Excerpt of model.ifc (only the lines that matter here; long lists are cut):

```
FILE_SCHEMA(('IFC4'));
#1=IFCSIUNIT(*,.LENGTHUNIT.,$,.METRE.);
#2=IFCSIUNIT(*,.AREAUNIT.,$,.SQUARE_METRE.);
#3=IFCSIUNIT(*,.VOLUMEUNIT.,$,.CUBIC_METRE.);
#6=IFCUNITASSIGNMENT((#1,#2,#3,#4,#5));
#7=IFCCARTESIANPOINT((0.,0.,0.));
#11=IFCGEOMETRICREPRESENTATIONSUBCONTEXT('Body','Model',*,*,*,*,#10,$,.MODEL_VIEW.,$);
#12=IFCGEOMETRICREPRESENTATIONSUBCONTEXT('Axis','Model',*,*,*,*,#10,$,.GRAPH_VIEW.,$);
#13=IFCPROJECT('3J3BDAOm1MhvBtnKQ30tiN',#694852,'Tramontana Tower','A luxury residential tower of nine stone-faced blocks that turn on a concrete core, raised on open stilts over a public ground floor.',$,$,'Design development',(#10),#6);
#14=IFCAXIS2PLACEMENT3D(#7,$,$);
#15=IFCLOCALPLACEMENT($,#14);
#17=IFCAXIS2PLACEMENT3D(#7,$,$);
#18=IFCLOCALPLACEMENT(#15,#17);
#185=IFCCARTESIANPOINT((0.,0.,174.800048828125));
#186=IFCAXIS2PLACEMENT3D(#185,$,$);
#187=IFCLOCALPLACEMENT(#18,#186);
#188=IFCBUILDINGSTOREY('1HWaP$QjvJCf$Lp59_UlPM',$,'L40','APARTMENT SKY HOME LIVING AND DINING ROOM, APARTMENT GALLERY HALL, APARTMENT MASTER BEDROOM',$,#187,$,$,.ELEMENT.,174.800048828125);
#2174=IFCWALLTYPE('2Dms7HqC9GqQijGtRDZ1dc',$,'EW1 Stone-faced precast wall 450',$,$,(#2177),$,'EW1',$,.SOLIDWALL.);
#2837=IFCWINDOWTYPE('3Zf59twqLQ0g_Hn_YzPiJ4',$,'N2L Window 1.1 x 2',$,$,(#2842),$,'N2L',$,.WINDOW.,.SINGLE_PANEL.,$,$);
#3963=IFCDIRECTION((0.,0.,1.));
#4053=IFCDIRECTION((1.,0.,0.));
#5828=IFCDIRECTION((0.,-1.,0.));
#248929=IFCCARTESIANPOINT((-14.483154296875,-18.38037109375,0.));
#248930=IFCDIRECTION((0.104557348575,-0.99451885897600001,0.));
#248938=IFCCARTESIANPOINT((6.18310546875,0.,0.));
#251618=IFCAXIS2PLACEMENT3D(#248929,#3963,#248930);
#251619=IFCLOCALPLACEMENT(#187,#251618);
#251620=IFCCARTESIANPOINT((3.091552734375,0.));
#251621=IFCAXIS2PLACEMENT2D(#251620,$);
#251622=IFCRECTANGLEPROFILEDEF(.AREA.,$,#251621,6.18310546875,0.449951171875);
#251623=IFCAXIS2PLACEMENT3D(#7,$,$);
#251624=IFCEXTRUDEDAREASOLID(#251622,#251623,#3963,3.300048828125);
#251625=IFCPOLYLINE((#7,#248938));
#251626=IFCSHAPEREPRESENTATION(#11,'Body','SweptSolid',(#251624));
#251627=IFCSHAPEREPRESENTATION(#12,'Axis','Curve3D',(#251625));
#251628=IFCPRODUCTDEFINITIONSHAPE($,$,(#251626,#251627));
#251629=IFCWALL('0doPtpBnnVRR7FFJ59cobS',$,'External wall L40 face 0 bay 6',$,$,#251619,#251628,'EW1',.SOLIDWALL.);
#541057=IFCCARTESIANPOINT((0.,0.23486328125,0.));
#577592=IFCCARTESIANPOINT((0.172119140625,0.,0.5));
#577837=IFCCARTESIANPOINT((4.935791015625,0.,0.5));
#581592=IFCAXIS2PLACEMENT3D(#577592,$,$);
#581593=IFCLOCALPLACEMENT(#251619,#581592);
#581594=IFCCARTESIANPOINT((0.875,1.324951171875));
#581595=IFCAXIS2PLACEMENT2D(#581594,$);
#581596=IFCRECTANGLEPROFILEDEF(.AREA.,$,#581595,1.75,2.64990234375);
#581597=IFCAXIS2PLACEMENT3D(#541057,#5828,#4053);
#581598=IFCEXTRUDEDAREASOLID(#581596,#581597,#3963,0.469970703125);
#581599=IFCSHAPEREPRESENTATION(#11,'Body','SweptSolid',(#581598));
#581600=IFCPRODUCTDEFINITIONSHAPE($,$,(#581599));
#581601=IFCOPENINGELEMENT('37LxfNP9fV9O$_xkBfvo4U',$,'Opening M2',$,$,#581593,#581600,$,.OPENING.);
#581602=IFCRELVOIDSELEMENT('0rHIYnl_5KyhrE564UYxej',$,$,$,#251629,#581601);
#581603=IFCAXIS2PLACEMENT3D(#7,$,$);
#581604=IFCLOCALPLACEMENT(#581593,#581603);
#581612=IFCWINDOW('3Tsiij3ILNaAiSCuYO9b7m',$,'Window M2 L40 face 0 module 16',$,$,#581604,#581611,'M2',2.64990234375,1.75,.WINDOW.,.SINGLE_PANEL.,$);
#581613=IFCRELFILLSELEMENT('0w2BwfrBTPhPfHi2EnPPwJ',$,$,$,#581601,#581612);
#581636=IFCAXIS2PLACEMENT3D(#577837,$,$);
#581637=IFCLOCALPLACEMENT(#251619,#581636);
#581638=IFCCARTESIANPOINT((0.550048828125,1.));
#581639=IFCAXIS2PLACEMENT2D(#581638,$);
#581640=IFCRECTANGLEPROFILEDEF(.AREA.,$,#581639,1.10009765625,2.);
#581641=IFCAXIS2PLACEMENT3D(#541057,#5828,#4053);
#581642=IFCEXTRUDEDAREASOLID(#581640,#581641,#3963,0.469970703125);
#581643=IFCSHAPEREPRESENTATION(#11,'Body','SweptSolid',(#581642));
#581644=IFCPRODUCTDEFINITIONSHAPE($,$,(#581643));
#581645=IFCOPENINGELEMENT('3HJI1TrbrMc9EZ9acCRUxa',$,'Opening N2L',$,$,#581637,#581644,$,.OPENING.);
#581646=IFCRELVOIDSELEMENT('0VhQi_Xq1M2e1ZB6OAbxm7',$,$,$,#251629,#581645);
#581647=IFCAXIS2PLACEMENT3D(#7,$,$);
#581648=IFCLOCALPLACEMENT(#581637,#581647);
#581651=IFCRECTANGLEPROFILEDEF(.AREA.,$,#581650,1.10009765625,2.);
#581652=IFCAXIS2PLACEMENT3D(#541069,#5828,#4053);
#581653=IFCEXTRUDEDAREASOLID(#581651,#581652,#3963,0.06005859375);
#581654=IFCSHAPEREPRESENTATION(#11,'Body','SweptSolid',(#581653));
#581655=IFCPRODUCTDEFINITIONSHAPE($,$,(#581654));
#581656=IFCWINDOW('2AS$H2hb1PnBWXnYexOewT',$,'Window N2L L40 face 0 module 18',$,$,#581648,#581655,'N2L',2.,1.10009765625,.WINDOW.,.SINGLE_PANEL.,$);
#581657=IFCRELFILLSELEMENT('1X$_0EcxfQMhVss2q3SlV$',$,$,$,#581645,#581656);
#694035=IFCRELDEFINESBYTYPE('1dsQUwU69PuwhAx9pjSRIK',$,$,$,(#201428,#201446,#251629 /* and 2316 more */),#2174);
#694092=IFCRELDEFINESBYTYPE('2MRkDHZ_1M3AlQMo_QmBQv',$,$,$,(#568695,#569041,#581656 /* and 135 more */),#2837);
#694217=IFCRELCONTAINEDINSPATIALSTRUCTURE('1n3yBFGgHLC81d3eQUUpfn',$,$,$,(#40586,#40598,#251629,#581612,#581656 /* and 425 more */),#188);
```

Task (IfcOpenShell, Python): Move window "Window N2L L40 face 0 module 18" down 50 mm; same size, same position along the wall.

```python
import numpy as np
import ifcopenshell
import ifcopenshell.api.geometry
import ifcopenshell.util.placement
import ifcopenshell.util.unit

model = ifcopenshell.open("model.ifc")
unit_scale = ifcopenshell.util.unit.calculate_unit_scale(model)

window = model.by_id(581656)
opening = window.FillsVoids[0].RelatingOpeningElement
dz = -0.05

shift = np.array([0.0, 0.0, dz])
# The window is placed relative to its opening, so it follows when the opening moves.
matrix = ifcopenshell.util.placement.get_local_placement(opening.ObjectPlacement)
matrix[:3, 3] += shift
ifcopenshell.api.geometry.edit_object_placement(
    model, product=opening, matrix=matrix, is_si=False, should_transform_children=True
)

print(f"moved by {dz * unit_scale:+.3f} m")

model.write("model-out.ifc")
```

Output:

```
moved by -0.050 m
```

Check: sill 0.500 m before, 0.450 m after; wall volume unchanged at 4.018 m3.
